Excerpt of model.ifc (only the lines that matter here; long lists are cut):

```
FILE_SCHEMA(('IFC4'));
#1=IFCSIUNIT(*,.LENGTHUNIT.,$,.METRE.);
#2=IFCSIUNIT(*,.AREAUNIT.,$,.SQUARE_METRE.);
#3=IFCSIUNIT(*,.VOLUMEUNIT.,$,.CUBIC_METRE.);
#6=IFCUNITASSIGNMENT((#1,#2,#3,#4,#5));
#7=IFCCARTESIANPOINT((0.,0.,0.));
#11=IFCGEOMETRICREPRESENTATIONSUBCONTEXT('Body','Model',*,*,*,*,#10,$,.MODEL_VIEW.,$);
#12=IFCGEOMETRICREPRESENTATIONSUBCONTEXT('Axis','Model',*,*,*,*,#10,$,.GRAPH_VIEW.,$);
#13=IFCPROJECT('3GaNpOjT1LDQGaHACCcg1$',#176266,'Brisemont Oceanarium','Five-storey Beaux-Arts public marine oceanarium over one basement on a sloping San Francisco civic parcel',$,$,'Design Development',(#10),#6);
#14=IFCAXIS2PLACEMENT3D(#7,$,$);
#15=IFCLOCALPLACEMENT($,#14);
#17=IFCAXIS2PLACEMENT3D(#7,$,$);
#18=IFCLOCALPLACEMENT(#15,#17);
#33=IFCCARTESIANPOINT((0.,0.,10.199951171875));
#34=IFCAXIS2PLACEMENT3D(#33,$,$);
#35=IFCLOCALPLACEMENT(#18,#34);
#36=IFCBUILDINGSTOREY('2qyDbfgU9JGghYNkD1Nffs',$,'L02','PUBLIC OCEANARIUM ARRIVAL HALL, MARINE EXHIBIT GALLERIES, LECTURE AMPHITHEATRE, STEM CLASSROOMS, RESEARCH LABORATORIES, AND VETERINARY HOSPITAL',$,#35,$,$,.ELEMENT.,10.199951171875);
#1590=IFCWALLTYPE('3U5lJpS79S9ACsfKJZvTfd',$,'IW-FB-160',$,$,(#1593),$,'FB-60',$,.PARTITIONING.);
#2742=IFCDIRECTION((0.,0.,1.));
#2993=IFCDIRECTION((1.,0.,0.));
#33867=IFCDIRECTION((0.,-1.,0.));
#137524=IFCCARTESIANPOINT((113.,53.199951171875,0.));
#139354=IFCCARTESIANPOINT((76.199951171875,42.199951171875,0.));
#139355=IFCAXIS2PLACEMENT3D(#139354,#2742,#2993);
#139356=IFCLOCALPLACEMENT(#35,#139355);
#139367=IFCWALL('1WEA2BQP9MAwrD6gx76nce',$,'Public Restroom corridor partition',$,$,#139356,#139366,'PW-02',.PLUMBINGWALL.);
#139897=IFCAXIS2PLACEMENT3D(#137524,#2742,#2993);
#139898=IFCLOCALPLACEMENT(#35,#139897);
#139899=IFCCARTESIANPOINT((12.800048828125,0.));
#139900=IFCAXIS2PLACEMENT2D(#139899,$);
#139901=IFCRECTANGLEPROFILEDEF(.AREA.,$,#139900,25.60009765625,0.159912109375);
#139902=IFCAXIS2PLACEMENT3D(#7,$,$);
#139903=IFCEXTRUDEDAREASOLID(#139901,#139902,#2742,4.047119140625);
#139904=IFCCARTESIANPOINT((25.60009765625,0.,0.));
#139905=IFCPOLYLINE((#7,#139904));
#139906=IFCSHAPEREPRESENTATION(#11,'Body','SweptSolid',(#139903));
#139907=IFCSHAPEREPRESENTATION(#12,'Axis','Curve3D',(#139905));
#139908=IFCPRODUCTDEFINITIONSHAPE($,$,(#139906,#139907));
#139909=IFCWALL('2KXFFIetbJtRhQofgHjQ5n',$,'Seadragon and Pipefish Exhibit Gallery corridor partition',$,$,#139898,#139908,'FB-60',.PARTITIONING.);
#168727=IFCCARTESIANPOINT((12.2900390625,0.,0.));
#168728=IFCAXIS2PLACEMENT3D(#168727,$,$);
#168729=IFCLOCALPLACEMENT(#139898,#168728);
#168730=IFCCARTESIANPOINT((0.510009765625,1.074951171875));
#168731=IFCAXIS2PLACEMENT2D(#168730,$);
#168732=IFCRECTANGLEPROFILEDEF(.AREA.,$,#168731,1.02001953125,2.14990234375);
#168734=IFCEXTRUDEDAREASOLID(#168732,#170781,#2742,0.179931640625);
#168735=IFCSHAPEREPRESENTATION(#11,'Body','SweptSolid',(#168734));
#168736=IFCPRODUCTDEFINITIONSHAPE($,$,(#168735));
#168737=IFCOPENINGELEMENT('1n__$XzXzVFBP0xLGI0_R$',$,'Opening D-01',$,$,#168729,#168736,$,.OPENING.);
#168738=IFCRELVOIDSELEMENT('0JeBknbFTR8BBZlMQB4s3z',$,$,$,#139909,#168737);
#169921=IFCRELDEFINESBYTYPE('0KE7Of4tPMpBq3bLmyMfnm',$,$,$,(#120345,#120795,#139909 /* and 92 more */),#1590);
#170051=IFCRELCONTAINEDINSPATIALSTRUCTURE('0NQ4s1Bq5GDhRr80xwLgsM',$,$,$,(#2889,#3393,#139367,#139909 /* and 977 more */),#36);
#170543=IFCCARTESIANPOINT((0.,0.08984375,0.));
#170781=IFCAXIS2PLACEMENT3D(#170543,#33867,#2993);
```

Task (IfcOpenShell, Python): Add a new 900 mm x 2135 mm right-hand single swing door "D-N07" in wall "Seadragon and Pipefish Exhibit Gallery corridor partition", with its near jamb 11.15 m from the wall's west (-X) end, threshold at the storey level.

```python
import numpy as np
import ifcopenshell
import ifcopenshell.api.feature
import ifcopenshell.api.geometry
import ifcopenshell.api.root
import ifcopenshell.api.spatial
import ifcopenshell.geom
import ifcopenshell.util.element
import ifcopenshell.util.placement
import ifcopenshell.util.representation
import ifcopenshell.util.shape
import ifcopenshell.util.unit

model = ifcopenshell.open("model.ifc")
unit_scale = ifcopenshell.util.unit.calculate_unit_scale(model)
settings = ifcopenshell.geom.settings()


def volume(element):
    """Net volume in cubic metres, openings subtracted."""
    shape = ifcopenshell.geom.create_shape(settings, element)
    return ifcopenshell.util.shape.get_volume(shape.geometry)


wall = model.by_guid("2KXFFIetbJtRhQofgHjQ5n")
storey = ifcopenshell.util.element.get_container(wall, ifc_class="IfcBuildingStorey")
context = ifcopenshell.util.representation.get_context(model, "Model", "Body", "MODEL_VIEW")
before = volume(wall)

width, height, from_end, sill = 0.9, 2.135, 11.15, 0.0  # metres

# The wall runs along its own X axis, and the end named is its -X end.
wall_shape = ifcopenshell.geom.create_shape(settings, wall)
x, y, z = ifcopenshell.util.shape.get_vertices(wall_shape.geometry).T
start = x.min() + from_end
face, thickness = float(y.min()), float(y.max() - y.min())
wall_matrix = ifcopenshell.util.placement.get_local_placement(wall.ObjectPlacement)
level = ifcopenshell.util.placement.get_local_placement(storey.ObjectPlacement)[2, 3]


def in_wall(x, y):
    """Placement at x, y metres in the wall's axes, at sill height."""
    matrix = wall_matrix.copy()
    matrix[:, 3] = wall_matrix @ np.array([x / unit_scale, y / unit_scale, 0.0, 1.0])
    matrix[2, 3] = level + sill / unit_scale
    return matrix


# Opening: a box that overshoots both wall faces by 50 mm.
opening = ifcopenshell.api.root.create_entity(model, ifc_class="IfcOpeningElement", predefined_type="OPENING")
box = ifcopenshell.api.geometry.add_wall_representation(
    model, context=context, length=width, height=height, thickness=thickness + 0.1
)
ifcopenshell.api.geometry.assign_representation(model, product=opening, representation=box)
ifcopenshell.api.geometry.edit_object_placement(model, product=opening, matrix=in_wall(start, face - 0.05), is_si=False)
ifcopenshell.api.feature.add_feature(model, feature=opening, element=wall)

door = ifcopenshell.api.root.create_entity(model, ifc_class="IfcDoor", name="D-N07", predefined_type="DOOR")
door.OverallWidth, door.OverallHeight = width / unit_scale, height / unit_scale
door.OperationType = "SINGLE_SWING_RIGHT"
body = ifcopenshell.api.geometry.add_door_representation(
    model,
    context=context,
    overall_width=door.OverallWidth,
    overall_height=door.OverallHeight,
    operation_type="SINGLE_SWING_RIGHT",
    lining_properties={"LiningDepth": thickness / unit_scale, "ThresholdDepth": thickness / unit_scale},
)
ifcopenshell.api.geometry.assign_representation(model, product=door, representation=body)
ifcopenshell.api.spatial.assign_container(model, products=[door], relating_structure=storey)
ifcopenshell.api.feature.add_filling(model, opening=opening, element=door)

# The lining spans the wall, so the door starts at the wall face.
ifcopenshell.api.geometry.edit_object_placement(model, product=door, matrix=in_wall(start, face), is_si=False)

after = volume(wall)

print(f"wall volume {before:.3f} -> {after:.3f} m3")

model.write("model_updated.ifc")
```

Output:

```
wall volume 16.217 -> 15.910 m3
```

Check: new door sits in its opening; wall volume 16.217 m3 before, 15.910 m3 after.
